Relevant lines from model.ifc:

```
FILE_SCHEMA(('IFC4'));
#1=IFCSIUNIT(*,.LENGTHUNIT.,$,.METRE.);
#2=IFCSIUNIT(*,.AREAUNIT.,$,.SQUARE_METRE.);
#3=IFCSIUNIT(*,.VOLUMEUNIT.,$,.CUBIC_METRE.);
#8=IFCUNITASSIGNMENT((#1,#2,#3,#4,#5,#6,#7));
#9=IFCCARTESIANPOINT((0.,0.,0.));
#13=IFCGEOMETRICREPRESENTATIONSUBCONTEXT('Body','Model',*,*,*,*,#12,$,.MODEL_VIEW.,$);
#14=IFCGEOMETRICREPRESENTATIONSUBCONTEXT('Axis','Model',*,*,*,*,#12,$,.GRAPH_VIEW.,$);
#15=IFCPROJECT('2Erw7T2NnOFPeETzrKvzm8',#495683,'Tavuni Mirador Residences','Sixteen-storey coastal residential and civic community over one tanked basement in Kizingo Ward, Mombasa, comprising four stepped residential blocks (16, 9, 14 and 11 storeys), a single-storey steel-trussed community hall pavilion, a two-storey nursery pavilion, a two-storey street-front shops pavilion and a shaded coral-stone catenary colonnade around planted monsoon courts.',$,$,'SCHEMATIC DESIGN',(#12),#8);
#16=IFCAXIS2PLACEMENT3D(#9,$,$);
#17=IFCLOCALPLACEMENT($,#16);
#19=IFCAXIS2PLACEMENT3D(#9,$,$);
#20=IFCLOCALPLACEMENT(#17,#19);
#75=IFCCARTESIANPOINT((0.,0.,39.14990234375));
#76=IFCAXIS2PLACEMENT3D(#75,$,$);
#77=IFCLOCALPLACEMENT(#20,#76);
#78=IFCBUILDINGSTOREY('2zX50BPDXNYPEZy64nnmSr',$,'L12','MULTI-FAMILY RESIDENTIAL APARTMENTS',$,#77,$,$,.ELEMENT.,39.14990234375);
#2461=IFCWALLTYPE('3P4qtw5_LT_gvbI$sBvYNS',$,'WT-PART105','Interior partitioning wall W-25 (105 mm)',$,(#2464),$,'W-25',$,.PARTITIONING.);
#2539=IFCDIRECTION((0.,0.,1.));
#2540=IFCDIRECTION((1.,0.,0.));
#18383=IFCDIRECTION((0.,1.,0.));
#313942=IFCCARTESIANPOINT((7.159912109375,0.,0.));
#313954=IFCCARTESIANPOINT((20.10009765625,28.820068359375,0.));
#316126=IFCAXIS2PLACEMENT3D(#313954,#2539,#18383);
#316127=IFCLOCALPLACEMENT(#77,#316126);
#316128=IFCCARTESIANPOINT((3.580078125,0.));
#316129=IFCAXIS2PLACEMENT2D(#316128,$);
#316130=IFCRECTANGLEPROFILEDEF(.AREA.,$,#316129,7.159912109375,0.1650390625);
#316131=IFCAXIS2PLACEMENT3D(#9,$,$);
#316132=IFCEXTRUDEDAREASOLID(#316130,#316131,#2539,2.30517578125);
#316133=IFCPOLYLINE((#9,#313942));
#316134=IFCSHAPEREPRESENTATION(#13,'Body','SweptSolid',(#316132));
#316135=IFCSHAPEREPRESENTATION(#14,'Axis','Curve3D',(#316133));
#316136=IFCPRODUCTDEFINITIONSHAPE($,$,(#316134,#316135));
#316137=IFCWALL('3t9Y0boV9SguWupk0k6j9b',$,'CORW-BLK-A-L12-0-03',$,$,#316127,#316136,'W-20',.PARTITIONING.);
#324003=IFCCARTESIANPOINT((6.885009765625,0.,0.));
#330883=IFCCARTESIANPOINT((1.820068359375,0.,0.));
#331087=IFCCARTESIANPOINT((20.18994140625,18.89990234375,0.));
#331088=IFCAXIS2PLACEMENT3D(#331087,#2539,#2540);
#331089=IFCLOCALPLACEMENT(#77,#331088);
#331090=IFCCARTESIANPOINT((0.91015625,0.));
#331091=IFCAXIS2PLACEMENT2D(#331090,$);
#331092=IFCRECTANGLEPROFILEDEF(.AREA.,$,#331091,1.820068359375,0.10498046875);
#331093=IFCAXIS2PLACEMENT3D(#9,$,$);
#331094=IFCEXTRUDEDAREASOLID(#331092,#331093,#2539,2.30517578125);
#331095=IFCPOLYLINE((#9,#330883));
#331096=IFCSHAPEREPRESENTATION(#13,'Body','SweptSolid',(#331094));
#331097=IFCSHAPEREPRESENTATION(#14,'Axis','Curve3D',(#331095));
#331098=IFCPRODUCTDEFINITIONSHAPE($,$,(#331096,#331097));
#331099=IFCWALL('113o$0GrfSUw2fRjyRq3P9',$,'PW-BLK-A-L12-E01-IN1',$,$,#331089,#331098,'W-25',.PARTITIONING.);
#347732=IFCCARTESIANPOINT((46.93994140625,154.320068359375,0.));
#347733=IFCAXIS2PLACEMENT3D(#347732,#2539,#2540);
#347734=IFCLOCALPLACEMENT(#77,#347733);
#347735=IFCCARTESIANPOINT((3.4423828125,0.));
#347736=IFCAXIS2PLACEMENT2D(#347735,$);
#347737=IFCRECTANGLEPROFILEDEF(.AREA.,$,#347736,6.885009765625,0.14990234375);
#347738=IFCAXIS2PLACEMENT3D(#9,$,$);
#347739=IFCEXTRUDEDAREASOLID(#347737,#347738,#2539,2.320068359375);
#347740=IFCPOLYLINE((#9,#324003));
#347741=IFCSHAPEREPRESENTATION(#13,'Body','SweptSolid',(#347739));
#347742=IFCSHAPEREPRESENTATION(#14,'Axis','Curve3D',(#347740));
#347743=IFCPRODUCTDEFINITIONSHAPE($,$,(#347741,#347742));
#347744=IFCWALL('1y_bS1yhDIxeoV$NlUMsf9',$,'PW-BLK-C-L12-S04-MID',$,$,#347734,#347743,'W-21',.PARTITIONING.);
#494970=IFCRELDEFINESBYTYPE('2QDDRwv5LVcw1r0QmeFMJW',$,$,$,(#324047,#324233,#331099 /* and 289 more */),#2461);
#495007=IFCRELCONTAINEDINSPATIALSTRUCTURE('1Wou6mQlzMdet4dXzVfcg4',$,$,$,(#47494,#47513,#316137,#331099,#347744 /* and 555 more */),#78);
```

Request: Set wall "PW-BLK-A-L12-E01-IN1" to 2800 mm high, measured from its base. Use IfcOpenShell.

```python
import ifcopenshell
import ifcopenshell.geom
import ifcopenshell.util.representation
import ifcopenshell.util.shape
import ifcopenshell.util.unit

model = ifcopenshell.open("model.ifc")
unit_scale = ifcopenshell.util.unit.calculate_unit_scale(model)
settings = ifcopenshell.geom.settings()


def volume(element):
    """Net volume in cubic metres, openings subtracted."""
    shape = ifcopenshell.geom.create_shape(settings, element)
    return ifcopenshell.util.shape.get_volume(shape.geometry)


wall = model.by_id(331099)
before = volume(wall)

body = ifcopenshell.util.representation.get_representation(wall, "Model", "Body")
solid = body.Items[0]
old_height = solid.Depth
solid.Depth = 2.8 / unit_scale
after = volume(wall)

print(f"height {old_height:g} -> {solid.Depth:g}, volume {before:.3f} -> {after:.3f} m3")

model.write("model-out.ifc")
```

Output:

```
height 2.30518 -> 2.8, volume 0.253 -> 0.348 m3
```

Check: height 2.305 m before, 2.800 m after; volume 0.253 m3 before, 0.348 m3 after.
